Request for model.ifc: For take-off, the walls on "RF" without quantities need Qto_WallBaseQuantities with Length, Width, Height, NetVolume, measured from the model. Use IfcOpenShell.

First a look at what the model holds.

```python
import ifcopenshell
import ifcopenshell.util.element
import ifcopenshell.util.unit

model = ifcopenshell.open("model.ifc")
print(model.schema)
for unit_type in ("LENGTHUNIT", "AREAUNIT", "VOLUMEUNIT"):
    print(unit_type, ifcopenshell.util.unit.calculate_unit_scale(model, unit_type))
storey = next(s for s in model.by_type("IfcBuildingStorey") if s.Name == "RF")
walls = [e for e in ifcopenshell.util.element.get_decomposition(storey) if e.is_a("IfcWall")]
for e in sorted(walls, key=lambda e: e.id()):
    print(e.id(), e.is_a(), e.Name, list(ifcopenshell.util.element.get_psets(e, qtos_only=True)), sep=" | ")
```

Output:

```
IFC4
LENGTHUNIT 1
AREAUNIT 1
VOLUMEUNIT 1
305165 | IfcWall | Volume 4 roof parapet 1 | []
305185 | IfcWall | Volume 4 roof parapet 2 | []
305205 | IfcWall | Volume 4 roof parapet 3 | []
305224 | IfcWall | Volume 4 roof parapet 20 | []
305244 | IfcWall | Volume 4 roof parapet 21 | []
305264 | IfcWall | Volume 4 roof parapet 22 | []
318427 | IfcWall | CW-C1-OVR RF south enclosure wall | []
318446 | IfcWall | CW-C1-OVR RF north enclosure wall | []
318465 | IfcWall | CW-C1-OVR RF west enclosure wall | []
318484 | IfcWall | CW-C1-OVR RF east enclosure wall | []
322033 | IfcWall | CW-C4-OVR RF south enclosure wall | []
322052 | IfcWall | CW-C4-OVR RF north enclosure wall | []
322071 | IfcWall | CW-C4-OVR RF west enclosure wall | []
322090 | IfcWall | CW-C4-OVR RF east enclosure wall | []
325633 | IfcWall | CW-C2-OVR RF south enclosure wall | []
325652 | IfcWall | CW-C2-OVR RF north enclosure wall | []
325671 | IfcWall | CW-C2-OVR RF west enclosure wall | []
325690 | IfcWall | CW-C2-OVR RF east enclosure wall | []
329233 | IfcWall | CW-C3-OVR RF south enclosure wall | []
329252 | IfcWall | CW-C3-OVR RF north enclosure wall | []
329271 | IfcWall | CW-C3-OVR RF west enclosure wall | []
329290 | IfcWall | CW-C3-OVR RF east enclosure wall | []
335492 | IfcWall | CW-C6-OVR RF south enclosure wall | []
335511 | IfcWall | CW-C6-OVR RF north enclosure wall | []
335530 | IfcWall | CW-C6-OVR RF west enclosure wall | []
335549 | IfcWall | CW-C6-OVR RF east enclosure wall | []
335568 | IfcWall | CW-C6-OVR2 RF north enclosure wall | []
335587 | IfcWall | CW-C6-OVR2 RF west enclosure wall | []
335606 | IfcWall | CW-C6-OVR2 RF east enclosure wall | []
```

```python
import ifcopenshell
import ifcopenshell.api.pset
import ifcopenshell.geom
import ifcopenshell.util.element
import ifcopenshell.util.shape
import ifcopenshell.util.unit

model = ifcopenshell.open("model.ifc")
unit_scale = ifcopenshell.util.unit.calculate_unit_scale(model)
volume_scale = ifcopenshell.util.unit.calculate_unit_scale(model, "VOLUMEUNIT")
settings = ifcopenshell.geom.settings()

storey = next(s for s in model.by_type("IfcBuildingStorey") if s.Name == "RF")
walls = [e for e in ifcopenshell.util.element.get_decomposition(storey) if e.is_a("IfcWall")]

for e in sorted(walls, key=lambda e: e.id()):
    if ifcopenshell.util.element.get_psets(e, qtos_only=True, should_inherit=False):
        continue
    # Geometry comes back in metres, in the element's own axes.
    shape = ifcopenshell.geom.create_shape(settings, e)
    values = {
        "Length": ifcopenshell.util.shape.get_x(shape.geometry) / unit_scale,
        "Width": ifcopenshell.util.shape.get_y(shape.geometry) / unit_scale,
        "Height": ifcopenshell.util.shape.get_z(shape.geometry) / unit_scale,
        "NetVolume": ifcopenshell.util.shape.get_volume(shape.geometry) / volume_scale,
    }
    qto = ifcopenshell.api.pset.add_qto(model, product=e, name="Qto_WallBaseQuantities")
    ifcopenshell.api.pset.edit_qto(model, qto=qto, properties=values)
    print(e.id(), {k: round(v, 3) for k, v in values.items()})

model.write("model_edited.ifc")
```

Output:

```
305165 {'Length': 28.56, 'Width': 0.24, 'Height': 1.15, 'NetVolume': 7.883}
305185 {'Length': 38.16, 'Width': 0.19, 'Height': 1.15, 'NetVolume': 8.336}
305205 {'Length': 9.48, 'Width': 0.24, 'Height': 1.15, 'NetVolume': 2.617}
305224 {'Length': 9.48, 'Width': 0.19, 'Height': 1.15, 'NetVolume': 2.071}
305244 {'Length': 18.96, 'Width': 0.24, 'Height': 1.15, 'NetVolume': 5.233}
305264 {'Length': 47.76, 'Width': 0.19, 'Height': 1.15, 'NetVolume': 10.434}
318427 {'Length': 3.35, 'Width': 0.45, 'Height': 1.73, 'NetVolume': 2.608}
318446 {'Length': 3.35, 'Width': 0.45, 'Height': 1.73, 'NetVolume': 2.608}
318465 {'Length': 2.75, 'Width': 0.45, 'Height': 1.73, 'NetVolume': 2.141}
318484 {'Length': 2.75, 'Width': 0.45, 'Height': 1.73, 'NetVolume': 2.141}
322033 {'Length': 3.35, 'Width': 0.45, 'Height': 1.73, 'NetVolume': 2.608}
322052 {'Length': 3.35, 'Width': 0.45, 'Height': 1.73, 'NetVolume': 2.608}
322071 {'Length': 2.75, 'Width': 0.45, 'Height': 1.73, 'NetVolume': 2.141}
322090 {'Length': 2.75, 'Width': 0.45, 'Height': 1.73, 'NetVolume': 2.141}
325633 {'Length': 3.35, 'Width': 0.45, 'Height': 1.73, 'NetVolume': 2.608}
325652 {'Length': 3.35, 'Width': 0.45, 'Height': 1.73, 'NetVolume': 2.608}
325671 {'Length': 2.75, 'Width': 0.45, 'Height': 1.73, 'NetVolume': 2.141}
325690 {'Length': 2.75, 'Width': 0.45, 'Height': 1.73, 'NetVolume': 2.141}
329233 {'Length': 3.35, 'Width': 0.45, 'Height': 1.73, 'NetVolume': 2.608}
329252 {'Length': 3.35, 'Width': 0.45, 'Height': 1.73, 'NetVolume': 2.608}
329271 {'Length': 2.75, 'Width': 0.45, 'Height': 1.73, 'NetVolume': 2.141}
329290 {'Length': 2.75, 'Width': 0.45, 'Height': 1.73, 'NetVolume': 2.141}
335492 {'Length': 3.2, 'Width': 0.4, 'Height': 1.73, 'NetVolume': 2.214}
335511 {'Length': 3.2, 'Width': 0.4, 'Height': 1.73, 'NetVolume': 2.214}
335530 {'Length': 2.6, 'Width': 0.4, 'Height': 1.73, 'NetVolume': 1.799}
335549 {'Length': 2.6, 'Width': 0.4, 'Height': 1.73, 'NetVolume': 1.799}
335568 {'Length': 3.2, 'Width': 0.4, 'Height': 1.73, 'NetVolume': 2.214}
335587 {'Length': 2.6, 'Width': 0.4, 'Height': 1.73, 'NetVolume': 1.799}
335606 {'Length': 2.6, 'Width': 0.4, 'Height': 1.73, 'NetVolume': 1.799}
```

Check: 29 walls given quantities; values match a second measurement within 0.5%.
